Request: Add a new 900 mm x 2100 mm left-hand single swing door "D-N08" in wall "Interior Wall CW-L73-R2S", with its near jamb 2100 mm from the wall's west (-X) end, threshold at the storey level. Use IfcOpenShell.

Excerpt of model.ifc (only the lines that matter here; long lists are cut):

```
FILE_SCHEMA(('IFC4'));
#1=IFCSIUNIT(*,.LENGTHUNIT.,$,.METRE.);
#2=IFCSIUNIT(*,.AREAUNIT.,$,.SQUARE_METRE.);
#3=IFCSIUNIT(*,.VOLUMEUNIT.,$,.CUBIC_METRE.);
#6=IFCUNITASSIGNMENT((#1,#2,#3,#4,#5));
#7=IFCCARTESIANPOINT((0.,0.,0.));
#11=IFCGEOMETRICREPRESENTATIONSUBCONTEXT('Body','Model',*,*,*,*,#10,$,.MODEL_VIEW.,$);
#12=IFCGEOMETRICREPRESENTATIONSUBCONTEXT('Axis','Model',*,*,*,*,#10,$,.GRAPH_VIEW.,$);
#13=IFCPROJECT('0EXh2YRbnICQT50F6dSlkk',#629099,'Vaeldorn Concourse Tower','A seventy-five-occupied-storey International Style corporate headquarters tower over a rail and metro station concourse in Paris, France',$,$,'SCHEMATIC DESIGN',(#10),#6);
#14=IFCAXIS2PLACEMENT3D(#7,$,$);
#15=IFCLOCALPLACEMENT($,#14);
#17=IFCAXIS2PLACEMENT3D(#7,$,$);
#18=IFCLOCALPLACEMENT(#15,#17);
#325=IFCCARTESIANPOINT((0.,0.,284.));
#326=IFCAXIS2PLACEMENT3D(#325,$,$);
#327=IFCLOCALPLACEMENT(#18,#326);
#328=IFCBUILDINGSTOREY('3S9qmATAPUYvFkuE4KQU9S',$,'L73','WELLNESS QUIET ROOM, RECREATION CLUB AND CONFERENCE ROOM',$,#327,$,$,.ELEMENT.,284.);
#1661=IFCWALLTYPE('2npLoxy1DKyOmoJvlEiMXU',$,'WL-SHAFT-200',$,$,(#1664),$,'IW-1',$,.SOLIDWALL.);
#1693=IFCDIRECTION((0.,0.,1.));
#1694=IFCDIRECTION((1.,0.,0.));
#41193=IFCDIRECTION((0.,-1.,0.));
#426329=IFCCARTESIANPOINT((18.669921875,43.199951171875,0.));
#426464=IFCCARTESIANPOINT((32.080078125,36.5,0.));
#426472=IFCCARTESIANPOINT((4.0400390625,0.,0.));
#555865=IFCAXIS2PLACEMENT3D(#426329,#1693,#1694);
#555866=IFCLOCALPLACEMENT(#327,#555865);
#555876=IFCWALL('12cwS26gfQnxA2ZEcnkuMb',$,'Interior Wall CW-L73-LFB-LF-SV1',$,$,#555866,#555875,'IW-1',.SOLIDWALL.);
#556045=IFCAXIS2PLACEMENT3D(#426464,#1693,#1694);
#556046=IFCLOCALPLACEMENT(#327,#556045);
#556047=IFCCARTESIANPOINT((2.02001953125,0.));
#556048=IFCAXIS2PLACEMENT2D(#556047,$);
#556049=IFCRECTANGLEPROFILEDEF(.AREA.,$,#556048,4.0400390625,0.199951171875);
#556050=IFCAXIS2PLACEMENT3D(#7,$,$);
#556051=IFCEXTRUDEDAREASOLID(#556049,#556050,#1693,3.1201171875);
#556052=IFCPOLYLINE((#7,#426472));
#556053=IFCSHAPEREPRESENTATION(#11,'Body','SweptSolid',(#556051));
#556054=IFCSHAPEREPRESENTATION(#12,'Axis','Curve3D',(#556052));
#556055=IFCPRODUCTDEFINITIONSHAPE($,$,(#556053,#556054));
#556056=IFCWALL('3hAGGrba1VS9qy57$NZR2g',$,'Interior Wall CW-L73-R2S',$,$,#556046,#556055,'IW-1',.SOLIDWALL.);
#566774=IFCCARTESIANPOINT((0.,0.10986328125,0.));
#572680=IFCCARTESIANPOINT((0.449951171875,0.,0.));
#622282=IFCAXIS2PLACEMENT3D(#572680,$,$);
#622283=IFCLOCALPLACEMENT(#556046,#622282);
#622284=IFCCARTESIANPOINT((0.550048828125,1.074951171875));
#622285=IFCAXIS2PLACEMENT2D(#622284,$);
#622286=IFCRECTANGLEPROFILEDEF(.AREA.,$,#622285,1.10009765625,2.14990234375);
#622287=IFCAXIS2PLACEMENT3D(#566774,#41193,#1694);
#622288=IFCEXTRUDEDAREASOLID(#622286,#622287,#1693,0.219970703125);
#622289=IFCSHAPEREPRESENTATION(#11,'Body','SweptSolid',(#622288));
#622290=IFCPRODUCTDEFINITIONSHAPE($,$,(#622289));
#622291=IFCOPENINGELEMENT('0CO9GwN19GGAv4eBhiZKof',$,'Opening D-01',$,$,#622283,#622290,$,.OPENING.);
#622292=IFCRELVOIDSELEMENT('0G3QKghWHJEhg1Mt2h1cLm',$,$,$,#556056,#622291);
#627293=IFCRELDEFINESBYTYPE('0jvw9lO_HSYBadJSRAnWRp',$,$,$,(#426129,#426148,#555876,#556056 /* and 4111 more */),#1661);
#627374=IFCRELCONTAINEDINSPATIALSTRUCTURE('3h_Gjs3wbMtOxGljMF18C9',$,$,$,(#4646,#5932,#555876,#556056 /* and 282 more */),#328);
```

```python
import numpy as np
import ifcopenshell
import ifcopenshell.api.feature
import ifcopenshell.api.geometry
import ifcopenshell.api.root
import ifcopenshell.api.spatial
import ifcopenshell.geom
import ifcopenshell.util.element
import ifcopenshell.util.placement
import ifcopenshell.util.representation
import ifcopenshell.util.shape
import ifcopenshell.util.unit

model = ifcopenshell.open("model.ifc")
unit_scale = ifcopenshell.util.unit.calculate_unit_scale(model)
settings = ifcopenshell.geom.settings()


def volume(element):
    """Net volume in cubic metres, openings subtracted."""
    shape = ifcopenshell.geom.create_shape(settings, element)
    return ifcopenshell.util.shape.get_volume(shape.geometry)


wall = model.by_id(556056)
storey = ifcopenshell.util.element.get_container(wall, ifc_class="IfcBuildingStorey")
context = ifcopenshell.util.representation.get_context(model, "Model", "Body", "MODEL_VIEW")
before = volume(wall)

width, height, from_end, sill = 0.9, 2.1, 2.1, 0.0  # metres

# The wall runs along its own X axis, and the end named is its -X end.
wall_shape = ifcopenshell.geom.create_shape(settings, wall)
x, y, z = ifcopenshell.util.shape.get_vertices(wall_shape.geometry).T
start = x.min() + from_end
face, thickness = float(y.min()), float(y.max() - y.min())
wall_matrix = ifcopenshell.util.placement.get_local_placement(wall.ObjectPlacement)
level = ifcopenshell.util.placement.get_local_placement(storey.ObjectPlacement)[2, 3]


def in_wall(x, y):
    """Placement at x, y metres in the wall's axes, at sill height."""
    matrix = wall_matrix.copy()
    matrix[:, 3] = wall_matrix @ np.array([x / unit_scale, y / unit_scale, 0.0, 1.0])
    matrix[2, 3] = level + sill / unit_scale
    return matrix


# Opening: a box that overshoots both wall faces by 50 mm.
opening = ifcopenshell.api.root.create_entity(model, ifc_class="IfcOpeningElement", predefined_type="OPENING")
box = ifcopenshell.api.geometry.add_wall_representation(
    model, context=context, length=width, height=height, thickness=thickness + 0.1
)
ifcopenshell.api.geometry.assign_representation(model, product=opening, representation=box)
ifcopenshell.api.geometry.edit_object_placement(model, product=opening, matrix=in_wall(start, face - 0.05), is_si=False)
ifcopenshell.api.feature.add_feature(model, feature=opening, element=wall)

door = ifcopenshell.api.root.create_entity(model, ifc_class="IfcDoor", name="D-N08", predefined_type="DOOR")
door.OverallWidth, door.OverallHeight = width / unit_scale, height / unit_scale
door.OperationType = "SINGLE_SWING_LEFT"
body = ifcopenshell.api.geometry.add_door_representation(
    model,
    context=context,
    overall_width=door.OverallWidth,
    overall_height=door.OverallHeight,
    operation_type="SINGLE_SWING_LEFT",
    lining_properties={"LiningDepth": thickness / unit_scale, "ThresholdDepth": thickness / unit_scale},
)
ifcopenshell.api.geometry.assign_representation(model, product=door, representation=body)
ifcopenshell.api.spatial.assign_container(model, products=[door], relating_structure=storey)
ifcopenshell.api.feature.add_filling(model, opening=opening, element=door)

# The lining spans the wall, so the door starts at the wall face.
ifcopenshell.api.geometry.edit_object_placement(model, product=door, matrix=in_wall(start, face), is_si=False)

after = volume(wall)

print(f"wall volume {before:.3f} -> {after:.3f} m3")

model.write("model_v2.ifc")
```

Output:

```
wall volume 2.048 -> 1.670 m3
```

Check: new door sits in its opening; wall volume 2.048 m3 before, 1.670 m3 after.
